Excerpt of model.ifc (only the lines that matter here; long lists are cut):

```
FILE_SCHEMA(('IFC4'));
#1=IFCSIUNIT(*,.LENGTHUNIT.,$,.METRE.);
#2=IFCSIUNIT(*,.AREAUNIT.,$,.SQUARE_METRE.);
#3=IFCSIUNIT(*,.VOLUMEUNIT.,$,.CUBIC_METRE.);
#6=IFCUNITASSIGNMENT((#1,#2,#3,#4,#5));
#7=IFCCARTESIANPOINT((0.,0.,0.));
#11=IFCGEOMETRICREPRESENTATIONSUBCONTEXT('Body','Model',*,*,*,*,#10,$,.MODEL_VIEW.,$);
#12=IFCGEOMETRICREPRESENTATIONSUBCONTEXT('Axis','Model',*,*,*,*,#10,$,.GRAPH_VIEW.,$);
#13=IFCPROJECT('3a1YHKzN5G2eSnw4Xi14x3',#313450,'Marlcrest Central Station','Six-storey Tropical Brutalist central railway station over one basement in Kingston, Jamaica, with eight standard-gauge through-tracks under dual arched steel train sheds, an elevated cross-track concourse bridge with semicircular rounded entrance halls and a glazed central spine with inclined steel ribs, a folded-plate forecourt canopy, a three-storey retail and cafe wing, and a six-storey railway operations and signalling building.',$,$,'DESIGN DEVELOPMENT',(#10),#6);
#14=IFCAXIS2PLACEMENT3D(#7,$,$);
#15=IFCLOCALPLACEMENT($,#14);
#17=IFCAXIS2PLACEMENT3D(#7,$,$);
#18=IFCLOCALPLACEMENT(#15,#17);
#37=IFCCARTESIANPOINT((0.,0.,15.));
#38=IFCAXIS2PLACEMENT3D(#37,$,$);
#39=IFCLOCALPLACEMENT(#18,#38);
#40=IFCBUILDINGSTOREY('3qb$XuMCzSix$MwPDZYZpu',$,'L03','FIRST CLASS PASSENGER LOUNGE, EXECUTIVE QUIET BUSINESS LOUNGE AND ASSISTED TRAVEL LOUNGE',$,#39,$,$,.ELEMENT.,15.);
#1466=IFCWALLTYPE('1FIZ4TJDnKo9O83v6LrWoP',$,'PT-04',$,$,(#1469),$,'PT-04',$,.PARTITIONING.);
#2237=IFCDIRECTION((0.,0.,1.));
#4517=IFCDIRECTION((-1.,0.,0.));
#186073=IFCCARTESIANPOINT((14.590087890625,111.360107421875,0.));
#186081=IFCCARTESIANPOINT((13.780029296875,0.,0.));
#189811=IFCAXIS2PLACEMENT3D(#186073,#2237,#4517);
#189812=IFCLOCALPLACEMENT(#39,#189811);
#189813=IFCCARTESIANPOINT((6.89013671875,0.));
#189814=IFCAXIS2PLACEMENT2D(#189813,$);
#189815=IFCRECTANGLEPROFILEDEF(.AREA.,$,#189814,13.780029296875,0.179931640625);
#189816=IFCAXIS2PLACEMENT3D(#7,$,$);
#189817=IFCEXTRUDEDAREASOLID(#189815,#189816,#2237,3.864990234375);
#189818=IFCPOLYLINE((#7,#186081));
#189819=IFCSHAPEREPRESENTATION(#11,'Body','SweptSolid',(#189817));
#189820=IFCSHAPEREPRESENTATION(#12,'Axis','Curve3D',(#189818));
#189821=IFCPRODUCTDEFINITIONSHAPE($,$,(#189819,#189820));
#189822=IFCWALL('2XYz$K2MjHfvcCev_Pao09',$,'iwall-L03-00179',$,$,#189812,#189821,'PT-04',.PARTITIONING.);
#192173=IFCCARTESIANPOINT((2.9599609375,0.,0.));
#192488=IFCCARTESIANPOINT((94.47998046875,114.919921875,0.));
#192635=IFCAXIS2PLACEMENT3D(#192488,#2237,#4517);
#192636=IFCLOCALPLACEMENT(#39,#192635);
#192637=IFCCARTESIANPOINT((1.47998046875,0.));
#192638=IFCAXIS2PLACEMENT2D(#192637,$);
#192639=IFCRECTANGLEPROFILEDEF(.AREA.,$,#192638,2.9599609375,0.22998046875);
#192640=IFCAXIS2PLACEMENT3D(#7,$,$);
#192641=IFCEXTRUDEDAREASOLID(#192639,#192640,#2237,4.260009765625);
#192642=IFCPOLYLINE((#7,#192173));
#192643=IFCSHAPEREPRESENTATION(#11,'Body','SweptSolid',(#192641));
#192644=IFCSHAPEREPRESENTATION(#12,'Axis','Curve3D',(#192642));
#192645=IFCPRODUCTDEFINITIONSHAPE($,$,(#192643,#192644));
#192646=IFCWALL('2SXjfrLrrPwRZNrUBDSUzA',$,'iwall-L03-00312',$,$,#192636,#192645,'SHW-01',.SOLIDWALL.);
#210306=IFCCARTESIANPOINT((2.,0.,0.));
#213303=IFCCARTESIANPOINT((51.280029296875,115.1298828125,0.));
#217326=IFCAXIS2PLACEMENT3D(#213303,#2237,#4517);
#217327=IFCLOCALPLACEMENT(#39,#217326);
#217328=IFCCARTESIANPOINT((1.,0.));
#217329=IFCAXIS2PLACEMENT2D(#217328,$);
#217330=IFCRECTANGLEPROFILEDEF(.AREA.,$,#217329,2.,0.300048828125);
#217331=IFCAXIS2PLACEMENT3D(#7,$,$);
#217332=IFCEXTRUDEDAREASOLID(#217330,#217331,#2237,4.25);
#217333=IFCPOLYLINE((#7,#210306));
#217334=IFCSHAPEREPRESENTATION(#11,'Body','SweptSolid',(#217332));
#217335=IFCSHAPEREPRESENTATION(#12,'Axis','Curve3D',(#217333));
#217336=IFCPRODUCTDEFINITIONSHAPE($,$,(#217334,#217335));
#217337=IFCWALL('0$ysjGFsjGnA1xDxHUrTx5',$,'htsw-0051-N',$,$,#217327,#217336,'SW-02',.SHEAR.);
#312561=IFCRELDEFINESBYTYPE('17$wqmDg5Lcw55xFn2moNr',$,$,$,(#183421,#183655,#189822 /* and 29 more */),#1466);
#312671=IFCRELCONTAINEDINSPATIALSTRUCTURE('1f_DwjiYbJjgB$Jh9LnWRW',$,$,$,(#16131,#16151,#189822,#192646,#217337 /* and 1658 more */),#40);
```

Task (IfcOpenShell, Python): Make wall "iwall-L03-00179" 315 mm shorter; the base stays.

```python
import ifcopenshell
import ifcopenshell.geom
import ifcopenshell.util.representation
import ifcopenshell.util.shape
import ifcopenshell.util.unit

model = ifcopenshell.open("model.ifc")
unit_scale = ifcopenshell.util.unit.calculate_unit_scale(model)
settings = ifcopenshell.geom.settings()


def volume(element):
    """Net volume in cubic metres, openings subtracted."""
    shape = ifcopenshell.geom.create_shape(settings, element)
    return ifcopenshell.util.shape.get_volume(shape.geometry)


wall = model.by_guid("2XYz$K2MjHfvcCev_Pao09")
before = volume(wall)

body = ifcopenshell.util.representation.get_representation(wall, "Model", "Body")
solid = body.Items[0]
old_height = solid.Depth
solid.Depth -= 0.315 / unit_scale
after = volume(wall)

print(f"height {old_height:g} -> {solid.Depth:g}, volume {before:.3f} -> {after:.3f} m3")

model.write("model-out.ifc")
```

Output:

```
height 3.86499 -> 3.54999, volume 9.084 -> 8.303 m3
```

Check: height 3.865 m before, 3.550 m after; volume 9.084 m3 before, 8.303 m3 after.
